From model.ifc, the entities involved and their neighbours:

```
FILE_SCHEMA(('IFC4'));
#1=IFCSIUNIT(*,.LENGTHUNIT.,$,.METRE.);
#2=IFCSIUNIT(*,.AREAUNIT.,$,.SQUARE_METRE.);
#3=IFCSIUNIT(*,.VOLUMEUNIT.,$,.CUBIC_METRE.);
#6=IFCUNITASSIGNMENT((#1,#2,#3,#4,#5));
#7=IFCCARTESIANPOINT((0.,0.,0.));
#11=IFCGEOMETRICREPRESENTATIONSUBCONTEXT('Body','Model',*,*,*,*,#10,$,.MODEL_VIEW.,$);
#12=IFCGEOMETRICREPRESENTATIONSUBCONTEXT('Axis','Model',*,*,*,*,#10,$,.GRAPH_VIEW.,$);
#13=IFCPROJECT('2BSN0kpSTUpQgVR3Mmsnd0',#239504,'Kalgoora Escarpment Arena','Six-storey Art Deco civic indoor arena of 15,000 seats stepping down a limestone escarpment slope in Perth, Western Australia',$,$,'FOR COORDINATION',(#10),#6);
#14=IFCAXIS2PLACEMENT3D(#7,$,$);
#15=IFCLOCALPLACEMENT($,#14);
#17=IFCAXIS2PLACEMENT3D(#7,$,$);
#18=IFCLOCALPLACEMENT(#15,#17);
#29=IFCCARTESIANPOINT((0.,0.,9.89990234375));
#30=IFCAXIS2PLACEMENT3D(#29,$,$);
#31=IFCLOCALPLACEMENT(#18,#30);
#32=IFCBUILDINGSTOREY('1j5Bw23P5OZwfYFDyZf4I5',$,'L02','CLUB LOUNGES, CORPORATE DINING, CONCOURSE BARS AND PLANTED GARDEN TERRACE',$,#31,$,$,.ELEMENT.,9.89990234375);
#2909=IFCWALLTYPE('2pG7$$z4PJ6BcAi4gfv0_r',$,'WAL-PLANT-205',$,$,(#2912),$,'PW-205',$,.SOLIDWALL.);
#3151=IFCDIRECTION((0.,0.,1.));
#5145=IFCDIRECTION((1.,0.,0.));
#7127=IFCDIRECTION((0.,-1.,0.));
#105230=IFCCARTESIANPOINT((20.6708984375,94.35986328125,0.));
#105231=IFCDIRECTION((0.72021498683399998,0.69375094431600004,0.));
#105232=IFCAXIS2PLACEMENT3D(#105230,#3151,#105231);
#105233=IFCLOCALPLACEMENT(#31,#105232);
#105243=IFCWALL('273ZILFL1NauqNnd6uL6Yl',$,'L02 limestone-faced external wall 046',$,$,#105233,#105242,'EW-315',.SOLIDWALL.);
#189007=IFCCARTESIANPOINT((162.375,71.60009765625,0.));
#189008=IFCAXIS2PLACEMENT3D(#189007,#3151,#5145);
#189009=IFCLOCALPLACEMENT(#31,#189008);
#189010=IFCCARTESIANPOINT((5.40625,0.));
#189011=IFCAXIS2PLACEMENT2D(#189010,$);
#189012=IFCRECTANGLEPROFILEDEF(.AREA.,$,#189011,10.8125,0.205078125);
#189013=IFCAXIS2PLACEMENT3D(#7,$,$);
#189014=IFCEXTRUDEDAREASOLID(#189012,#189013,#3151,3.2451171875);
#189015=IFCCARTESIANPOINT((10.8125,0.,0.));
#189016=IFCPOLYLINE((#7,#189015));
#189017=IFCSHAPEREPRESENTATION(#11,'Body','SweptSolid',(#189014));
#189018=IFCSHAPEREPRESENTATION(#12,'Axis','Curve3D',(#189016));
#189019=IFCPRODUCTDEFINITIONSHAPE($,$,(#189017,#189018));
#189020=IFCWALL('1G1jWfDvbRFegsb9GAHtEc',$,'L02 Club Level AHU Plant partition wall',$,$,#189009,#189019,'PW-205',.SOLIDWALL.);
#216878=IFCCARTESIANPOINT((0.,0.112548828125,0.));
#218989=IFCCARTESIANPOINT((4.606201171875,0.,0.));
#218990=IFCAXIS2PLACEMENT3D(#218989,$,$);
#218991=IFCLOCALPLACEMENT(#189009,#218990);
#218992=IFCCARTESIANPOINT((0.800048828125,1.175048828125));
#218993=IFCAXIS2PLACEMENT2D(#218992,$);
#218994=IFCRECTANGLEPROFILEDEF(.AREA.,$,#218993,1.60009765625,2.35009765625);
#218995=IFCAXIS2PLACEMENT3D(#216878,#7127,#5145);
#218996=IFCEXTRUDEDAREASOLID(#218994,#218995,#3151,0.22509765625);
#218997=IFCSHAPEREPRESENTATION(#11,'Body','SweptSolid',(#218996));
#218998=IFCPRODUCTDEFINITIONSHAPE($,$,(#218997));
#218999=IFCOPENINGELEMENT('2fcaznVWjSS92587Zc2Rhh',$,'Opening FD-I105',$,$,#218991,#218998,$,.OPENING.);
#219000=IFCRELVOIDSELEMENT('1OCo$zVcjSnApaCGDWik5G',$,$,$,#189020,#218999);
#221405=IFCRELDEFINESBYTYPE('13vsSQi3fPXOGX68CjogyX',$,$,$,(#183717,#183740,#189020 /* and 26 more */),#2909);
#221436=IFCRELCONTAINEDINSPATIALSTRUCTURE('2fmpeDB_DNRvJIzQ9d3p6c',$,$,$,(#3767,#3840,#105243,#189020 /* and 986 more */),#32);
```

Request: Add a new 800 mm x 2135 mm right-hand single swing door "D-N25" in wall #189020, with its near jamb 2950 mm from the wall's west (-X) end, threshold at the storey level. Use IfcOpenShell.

```python
import numpy as np
import ifcopenshell
import ifcopenshell.api.feature
import ifcopenshell.api.geometry
import ifcopenshell.api.root
import ifcopenshell.api.spatial
import ifcopenshell.geom
import ifcopenshell.util.element
import ifcopenshell.util.placement
import ifcopenshell.util.representation
import ifcopenshell.util.shape
import ifcopenshell.util.unit

model = ifcopenshell.open("model.ifc")
unit_scale = ifcopenshell.util.unit.calculate_unit_scale(model)
settings = ifcopenshell.geom.settings()


def volume(element):
    """Net volume in cubic metres, openings subtracted."""
    shape = ifcopenshell.geom.create_shape(settings, element)
    return ifcopenshell.util.shape.get_volume(shape.geometry)


wall = model.by_guid("1G1jWfDvbRFegsb9GAHtEc")
storey = ifcopenshell.util.element.get_container(wall, ifc_class="IfcBuildingStorey")
context = ifcopenshell.util.representation.get_context(model, "Model", "Body", "MODEL_VIEW")
before = volume(wall)

width, height, from_end, sill = 0.8, 2.135, 2.95, 0.0  # metres

# The wall runs along its own X axis, and the end named is its -X end.
wall_shape = ifcopenshell.geom.create_shape(settings, wall)
x, y, z = ifcopenshell.util.shape.get_vertices(wall_shape.geometry).T
start = x.min() + from_end
face, thickness = float(y.min()), float(y.max() - y.min())
wall_matrix = ifcopenshell.util.placement.get_local_placement(wall.ObjectPlacement)
level = ifcopenshell.util.placement.get_local_placement(storey.ObjectPlacement)[2, 3]


def in_wall(x, y):
    """Placement at x, y metres in the wall's axes, at sill height."""
    matrix = wall_matrix.copy()
    matrix[:, 3] = wall_matrix @ np.array([x / unit_scale, y / unit_scale, 0.0, 1.0])
    matrix[2, 3] = level + sill / unit_scale
    return matrix


# Opening: a box that overshoots both wall faces by 50 mm.
opening = ifcopenshell.api.root.create_entity(model, ifc_class="IfcOpeningElement", predefined_type="OPENING")
box = ifcopenshell.api.geometry.add_wall_representation(
    model, context=context, length=width, height=height, thickness=thickness + 0.1
)
ifcopenshell.api.geometry.assign_representation(model, product=opening, representation=box)
ifcopenshell.api.geometry.edit_object_placement(model, product=opening, matrix=in_wall(start, face - 0.05), is_si=False)
ifcopenshell.api.feature.add_feature(model, feature=opening, element=wall)

door = ifcopenshell.api.root.create_entity(model, ifc_class="IfcDoor", name="D-N25", predefined_type="DOOR")
door.OverallWidth, door.OverallHeight = width / unit_scale, height / unit_scale
door.OperationType = "SINGLE_SWING_RIGHT"
body = ifcopenshell.api.geometry.add_door_representation(
    model,
    context=context,
    overall_width=door.OverallWidth,
    overall_height=door.OverallHeight,
    operation_type="SINGLE_SWING_RIGHT",
    lining_properties={"LiningDepth": thickness / unit_scale, "ThresholdDepth": thickness / unit_scale},
)
ifcopenshell.api.geometry.assign_representation(model, product=door, representation=body)
ifcopenshell.api.spatial.assign_container(model, products=[door], relating_structure=storey)
ifcopenshell.api.feature.add_filling(model, opening=opening, element=door)

# The lining spans the wall, so the door starts at the wall face.
ifcopenshell.api.geometry.edit_object_placement(model, product=door, matrix=in_wall(start, face), is_si=False)

after = volume(wall)

print(f"wall volume {before:.3f} -> {after:.3f} m3")

model.write("model_rev.ifc")
```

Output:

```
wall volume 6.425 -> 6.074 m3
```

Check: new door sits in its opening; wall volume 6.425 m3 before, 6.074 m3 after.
